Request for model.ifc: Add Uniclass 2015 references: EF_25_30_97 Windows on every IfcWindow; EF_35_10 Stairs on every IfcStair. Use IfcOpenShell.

First a look at what the model holds.

```python
import ifcopenshell

model = ifcopenshell.open("model.ifc")
print(model.schema)
print("classifications:", [c.Name for c in model.by_type("IfcClassification")])
for ifc_class in ("IfcDoor", "IfcRoof", "IfcStair", "IfcWall", "IfcWindow"):
    print(ifc_class, len(model.by_type(ifc_class)))
```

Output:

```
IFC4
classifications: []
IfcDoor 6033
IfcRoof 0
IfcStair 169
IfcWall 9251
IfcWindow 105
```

```python
import ifcopenshell
import ifcopenshell.api.classification

model = ifcopenshell.open("model.ifc")

system = ifcopenshell.api.classification.add_classification(model, classification="Uniclass 2015")

codes = {
    "IfcWindow": ("EF_25_30_97", "Windows"),
    "IfcStair": ("EF_35_10", "Stairs"),
}
for ifc_class, (code, name) in codes.items():
    products = model.by_type(ifc_class)
    ifcopenshell.api.classification.add_reference(
        model, products=products, classification=system, identification=code, name=name
    )
    print(code, len(products))

model.write("model_v2.ifc")
```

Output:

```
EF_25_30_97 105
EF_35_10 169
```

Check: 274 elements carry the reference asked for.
